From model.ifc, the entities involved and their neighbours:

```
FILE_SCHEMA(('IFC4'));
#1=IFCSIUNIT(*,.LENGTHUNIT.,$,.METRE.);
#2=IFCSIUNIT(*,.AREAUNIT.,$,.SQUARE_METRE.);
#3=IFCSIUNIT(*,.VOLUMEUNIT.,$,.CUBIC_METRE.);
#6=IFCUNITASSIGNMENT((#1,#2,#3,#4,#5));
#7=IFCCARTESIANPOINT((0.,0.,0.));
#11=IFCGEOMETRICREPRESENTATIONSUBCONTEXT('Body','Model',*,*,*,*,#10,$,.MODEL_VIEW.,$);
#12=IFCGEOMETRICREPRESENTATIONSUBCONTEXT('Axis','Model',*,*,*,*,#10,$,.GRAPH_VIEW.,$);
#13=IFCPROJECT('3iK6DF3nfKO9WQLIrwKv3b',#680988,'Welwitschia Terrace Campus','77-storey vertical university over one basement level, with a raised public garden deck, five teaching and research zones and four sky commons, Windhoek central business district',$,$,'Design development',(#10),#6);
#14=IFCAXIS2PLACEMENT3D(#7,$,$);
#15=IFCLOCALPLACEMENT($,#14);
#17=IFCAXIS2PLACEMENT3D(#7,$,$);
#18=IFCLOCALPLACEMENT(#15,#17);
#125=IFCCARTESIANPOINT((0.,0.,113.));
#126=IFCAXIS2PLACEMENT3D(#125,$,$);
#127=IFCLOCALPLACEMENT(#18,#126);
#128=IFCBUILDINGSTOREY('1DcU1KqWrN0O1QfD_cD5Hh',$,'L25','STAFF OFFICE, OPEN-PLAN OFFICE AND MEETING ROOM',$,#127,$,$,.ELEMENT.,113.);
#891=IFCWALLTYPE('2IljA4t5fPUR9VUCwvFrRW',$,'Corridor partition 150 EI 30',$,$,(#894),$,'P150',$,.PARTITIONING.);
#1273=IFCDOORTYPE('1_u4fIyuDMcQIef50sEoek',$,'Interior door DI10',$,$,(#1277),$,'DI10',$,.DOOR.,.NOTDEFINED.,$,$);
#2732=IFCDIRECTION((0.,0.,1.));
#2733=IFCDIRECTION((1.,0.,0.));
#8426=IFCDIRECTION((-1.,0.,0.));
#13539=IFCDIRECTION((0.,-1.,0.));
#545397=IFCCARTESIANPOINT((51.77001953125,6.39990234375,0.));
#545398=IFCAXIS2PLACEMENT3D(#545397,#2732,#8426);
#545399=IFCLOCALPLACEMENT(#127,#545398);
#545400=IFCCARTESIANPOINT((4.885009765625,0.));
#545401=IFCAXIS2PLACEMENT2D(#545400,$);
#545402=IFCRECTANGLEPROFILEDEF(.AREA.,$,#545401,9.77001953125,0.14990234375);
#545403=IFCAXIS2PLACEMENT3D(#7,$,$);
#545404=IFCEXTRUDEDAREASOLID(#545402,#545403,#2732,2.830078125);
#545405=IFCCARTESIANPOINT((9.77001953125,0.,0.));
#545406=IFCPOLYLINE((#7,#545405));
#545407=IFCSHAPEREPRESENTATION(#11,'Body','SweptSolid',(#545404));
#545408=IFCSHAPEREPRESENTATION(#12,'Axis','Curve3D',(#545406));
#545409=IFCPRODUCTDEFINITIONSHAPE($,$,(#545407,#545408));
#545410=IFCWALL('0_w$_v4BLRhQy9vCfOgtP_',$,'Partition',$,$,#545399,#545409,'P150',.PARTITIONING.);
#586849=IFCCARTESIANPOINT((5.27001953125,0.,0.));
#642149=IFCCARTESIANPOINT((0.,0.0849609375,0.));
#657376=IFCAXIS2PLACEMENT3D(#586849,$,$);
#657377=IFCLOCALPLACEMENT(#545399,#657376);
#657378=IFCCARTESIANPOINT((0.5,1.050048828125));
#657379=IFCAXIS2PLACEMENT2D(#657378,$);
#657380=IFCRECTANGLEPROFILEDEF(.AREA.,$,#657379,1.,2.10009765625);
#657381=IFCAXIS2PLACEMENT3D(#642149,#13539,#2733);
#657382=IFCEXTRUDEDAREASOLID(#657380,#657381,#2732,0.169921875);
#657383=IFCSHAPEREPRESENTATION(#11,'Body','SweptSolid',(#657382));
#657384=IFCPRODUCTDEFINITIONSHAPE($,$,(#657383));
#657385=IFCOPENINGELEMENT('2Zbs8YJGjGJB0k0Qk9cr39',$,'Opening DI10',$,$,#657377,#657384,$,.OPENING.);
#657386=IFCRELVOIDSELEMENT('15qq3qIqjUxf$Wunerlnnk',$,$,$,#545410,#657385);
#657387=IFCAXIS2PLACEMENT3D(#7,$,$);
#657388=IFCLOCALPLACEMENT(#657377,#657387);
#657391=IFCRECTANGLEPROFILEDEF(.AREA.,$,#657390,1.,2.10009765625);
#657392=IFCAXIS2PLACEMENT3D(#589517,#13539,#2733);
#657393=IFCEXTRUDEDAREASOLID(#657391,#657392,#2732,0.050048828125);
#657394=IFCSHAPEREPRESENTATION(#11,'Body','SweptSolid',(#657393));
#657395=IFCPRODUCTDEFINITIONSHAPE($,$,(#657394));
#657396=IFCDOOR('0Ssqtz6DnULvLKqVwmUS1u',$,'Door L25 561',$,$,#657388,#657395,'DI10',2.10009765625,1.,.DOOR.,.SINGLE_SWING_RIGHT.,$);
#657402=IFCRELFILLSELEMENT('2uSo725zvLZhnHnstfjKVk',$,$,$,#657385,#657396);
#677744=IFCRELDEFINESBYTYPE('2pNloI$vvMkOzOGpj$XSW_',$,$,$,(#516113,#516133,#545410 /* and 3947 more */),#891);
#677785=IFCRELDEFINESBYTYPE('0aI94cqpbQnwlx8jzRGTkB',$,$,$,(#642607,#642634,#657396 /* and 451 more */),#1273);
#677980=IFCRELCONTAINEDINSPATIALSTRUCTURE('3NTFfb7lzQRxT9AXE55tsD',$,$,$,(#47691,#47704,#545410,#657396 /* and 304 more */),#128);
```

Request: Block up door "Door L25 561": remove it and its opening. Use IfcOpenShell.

```python
import ifcopenshell
import ifcopenshell.api.feature
import ifcopenshell.api.root
import ifcopenshell.geom
import ifcopenshell.util.shape

model = ifcopenshell.open("model.ifc")
settings = ifcopenshell.geom.settings()


def volume(element):
    """Net volume in cubic metres, openings subtracted."""
    shape = ifcopenshell.geom.create_shape(settings, element)
    return ifcopenshell.util.shape.get_volume(shape.geometry)


door = model.by_guid("0Ssqtz6DnULvLKqVwmUS1u")
opening = door.FillsVoids[0].RelatingOpeningElement
wall = opening.VoidsElements[0].RelatingBuildingElement
before = volume(wall)

ifcopenshell.api.root.remove_product(model, product=door)
ifcopenshell.api.feature.remove_feature(model, feature=opening)

after = volume(wall)

print(f"wall volume {before:.3f} -> {after:.3f} m3")

model.write("model_edited.ifc")
```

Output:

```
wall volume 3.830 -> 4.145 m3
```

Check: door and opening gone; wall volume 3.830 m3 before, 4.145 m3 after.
